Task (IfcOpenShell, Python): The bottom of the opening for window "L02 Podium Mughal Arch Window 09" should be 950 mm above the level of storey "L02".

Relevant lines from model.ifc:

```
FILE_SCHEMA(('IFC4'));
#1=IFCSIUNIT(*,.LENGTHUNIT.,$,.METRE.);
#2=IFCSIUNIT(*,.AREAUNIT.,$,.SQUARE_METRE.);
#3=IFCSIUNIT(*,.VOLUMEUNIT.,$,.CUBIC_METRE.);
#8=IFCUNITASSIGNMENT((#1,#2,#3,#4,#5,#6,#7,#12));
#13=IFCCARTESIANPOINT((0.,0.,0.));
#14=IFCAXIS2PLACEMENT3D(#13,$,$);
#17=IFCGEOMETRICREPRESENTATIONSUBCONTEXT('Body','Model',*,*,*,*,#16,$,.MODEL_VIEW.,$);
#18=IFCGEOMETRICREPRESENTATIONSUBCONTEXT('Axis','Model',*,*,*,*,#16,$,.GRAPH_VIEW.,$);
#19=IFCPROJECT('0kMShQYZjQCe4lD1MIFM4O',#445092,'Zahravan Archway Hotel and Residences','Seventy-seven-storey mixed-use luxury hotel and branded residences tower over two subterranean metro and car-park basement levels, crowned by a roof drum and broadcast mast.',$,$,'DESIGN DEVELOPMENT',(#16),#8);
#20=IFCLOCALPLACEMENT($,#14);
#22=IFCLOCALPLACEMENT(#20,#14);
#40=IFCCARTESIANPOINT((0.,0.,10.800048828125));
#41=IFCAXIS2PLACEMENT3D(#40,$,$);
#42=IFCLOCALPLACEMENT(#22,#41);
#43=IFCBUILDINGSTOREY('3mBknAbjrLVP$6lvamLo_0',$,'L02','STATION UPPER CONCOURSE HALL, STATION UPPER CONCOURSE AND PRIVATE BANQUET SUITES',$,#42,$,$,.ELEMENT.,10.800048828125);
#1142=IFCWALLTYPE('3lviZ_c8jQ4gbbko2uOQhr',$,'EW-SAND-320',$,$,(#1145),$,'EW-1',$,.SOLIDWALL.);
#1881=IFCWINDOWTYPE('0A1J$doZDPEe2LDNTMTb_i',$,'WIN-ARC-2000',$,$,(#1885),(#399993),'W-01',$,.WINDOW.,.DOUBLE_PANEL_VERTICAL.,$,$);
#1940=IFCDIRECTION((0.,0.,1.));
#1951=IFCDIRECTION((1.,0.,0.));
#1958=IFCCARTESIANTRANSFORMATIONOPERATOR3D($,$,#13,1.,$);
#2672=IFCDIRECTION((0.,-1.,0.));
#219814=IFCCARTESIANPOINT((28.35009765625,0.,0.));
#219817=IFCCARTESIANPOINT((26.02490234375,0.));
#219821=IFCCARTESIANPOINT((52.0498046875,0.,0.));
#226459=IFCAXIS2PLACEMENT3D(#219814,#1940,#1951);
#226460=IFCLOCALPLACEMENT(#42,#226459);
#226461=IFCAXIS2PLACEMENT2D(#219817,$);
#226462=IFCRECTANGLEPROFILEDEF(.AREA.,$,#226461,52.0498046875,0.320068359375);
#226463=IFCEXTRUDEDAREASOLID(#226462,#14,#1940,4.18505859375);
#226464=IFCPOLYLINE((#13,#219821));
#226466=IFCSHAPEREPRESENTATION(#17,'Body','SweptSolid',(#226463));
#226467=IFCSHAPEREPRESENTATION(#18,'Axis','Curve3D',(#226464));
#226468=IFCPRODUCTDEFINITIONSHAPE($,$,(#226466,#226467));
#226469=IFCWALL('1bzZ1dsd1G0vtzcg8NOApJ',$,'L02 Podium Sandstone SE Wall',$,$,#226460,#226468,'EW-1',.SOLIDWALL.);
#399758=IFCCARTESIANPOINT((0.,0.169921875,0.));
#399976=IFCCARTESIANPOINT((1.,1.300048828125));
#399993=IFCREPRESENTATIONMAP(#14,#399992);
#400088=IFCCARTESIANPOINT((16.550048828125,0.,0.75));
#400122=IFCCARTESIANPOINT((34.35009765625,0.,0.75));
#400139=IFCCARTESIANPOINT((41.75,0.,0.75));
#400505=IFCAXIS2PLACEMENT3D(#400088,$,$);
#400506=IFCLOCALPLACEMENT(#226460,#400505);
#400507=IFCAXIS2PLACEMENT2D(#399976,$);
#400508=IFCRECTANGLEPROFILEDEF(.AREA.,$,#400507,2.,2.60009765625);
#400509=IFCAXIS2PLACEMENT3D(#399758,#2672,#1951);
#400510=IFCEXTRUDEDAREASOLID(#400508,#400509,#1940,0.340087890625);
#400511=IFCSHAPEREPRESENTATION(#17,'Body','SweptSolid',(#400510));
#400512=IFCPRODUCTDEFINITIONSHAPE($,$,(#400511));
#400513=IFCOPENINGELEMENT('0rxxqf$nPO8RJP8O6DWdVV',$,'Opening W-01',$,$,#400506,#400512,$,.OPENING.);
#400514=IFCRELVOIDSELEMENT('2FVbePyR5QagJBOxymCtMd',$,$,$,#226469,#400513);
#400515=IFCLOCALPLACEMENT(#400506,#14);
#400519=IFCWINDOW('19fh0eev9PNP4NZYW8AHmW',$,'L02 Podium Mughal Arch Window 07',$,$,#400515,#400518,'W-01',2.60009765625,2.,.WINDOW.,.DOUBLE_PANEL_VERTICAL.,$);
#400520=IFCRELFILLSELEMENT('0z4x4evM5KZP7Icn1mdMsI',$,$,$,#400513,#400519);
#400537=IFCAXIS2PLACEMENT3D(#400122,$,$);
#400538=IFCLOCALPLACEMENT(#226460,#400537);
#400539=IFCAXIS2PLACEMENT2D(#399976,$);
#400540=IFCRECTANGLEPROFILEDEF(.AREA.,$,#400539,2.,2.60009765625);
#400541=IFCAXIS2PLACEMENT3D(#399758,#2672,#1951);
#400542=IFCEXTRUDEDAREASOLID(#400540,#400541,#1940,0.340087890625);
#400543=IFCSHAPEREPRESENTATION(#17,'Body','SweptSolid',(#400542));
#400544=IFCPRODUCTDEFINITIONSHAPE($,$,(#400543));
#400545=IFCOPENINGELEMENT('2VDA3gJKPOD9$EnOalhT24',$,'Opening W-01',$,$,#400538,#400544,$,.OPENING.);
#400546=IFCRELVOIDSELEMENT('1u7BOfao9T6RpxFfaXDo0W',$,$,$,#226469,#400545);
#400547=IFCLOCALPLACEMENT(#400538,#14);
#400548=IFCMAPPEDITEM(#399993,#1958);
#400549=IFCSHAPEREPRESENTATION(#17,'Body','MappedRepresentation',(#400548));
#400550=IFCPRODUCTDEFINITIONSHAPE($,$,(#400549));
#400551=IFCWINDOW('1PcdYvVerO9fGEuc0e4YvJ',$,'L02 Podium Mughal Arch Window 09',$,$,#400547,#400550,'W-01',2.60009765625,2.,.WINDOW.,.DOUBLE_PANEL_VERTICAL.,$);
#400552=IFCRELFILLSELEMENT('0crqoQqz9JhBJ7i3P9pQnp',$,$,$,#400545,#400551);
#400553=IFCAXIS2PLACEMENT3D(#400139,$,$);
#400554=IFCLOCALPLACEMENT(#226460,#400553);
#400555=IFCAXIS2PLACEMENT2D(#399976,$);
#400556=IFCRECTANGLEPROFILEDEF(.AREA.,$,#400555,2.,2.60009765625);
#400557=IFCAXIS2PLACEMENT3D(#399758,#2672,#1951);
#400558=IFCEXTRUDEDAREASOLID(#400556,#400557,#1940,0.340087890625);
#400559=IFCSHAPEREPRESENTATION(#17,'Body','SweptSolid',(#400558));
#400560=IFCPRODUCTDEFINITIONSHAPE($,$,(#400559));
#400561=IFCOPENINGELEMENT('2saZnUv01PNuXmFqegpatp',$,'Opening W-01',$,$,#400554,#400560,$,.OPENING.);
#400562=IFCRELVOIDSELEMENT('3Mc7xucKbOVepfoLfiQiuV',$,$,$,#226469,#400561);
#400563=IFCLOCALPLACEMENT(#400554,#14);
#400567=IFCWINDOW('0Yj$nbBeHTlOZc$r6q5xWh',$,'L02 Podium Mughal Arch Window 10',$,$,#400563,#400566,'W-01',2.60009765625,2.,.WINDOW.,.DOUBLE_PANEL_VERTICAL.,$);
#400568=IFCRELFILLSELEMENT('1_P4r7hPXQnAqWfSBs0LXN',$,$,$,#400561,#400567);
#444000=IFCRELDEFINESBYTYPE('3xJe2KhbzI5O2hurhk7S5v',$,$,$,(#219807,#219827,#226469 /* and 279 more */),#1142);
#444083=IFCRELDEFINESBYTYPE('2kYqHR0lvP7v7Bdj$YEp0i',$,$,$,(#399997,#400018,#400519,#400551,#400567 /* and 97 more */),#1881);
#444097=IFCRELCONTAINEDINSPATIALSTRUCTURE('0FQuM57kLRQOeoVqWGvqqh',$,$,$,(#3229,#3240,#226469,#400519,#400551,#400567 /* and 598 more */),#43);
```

```python
import numpy as np
import ifcopenshell
import ifcopenshell.api.geometry
import ifcopenshell.geom
import ifcopenshell.util.element
import ifcopenshell.util.placement
import ifcopenshell.util.shape
import ifcopenshell.util.unit

model = ifcopenshell.open("model.ifc")
unit_scale = ifcopenshell.util.unit.calculate_unit_scale(model)

window = model.by_id(400551)
opening = window.FillsVoids[0].RelatingOpeningElement
storey = ifcopenshell.util.element.get_container(window, ifc_class="IfcBuildingStorey")
level = ifcopenshell.util.placement.get_local_placement(storey.ObjectPlacement)[2, 3]

# The opening's origin need not be at the sill, so measure its lowest point.
shape = ifcopenshell.geom.create_shape(ifcopenshell.geom.settings(), opening)
bottom = ifcopenshell.util.shape.get_shape_bottom_elevation(shape, shape.geometry) / unit_scale
dz = level + 0.95 - bottom

shift = np.array([0.0, 0.0, dz])
# The window is placed relative to its opening, so it follows when the opening moves.
matrix = ifcopenshell.util.placement.get_local_placement(opening.ObjectPlacement)
matrix[:3, 3] += shift
ifcopenshell.api.geometry.edit_object_placement(
    model, product=opening, matrix=matrix, is_si=False, should_transform_children=True
)

print(f"moved by {dz * unit_scale:+.3f} m")

model.write("model_updated.ifc")
```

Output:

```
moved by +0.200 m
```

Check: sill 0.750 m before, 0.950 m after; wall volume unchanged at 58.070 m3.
